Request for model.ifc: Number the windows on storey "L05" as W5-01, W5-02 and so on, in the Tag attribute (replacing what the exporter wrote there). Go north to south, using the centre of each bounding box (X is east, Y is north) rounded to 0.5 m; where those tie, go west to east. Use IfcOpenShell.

First a look at what the model holds.

```python
import ifcopenshell
import ifcopenshell.util.element
import ifcopenshell.util.placement

model = ifcopenshell.open("model.ifc")
print(model.schema)
storey = next(s for s in model.by_type("IfcBuildingStorey") if s.Name == "L05")
windows = [e for e in ifcopenshell.util.element.get_decomposition(storey) if e.is_a("IfcWindow")]
for e in sorted(windows, key=lambda e: e.id()):
    origin = ifcopenshell.util.placement.get_local_placement(e.ObjectPlacement)[:3, 3]
    print(e.id(), e.Tag, e.Name, origin.round(2) + 0.0, sep=" | ")
```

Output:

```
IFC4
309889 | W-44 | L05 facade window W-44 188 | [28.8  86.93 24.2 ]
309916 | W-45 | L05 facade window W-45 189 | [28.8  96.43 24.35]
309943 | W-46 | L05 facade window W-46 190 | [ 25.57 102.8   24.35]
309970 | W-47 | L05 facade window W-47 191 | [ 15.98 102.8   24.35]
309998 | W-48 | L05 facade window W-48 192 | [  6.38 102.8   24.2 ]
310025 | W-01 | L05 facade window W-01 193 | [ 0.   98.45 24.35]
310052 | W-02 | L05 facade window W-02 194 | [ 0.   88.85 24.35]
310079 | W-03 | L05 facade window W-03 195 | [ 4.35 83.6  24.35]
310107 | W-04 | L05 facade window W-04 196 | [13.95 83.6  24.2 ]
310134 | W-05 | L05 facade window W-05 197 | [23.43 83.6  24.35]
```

```python
import ifcopenshell
import ifcopenshell.geom
import ifcopenshell.util.element
import ifcopenshell.util.shape

model = ifcopenshell.open("model.ifc")
settings = ifcopenshell.geom.settings()
settings.set("use-world-coords", True)


def centre(element):
    shape = ifcopenshell.geom.create_shape(settings, element)
    return ifcopenshell.util.shape.get_bbox_centroid(shape.geometry)


storey = next(s for s in model.by_type("IfcBuildingStorey") if s.Name == "L05")
windows = [e for e in ifcopenshell.util.element.get_decomposition(storey) if e.is_a("IfcWindow")]

# Insertion points can sit at a corner or the storey origin, so sort by the geometry (in metres).
centres = {e: centre(e) for e in windows}
windows.sort(key=lambda e: (-round(centres[e][1] / 0.5), centres[e][0]))

for i, e in enumerate(windows, start=1):
    number = f"W5-{i:02d}"
    e.Tag = number
    print(e.id(), number)

model.write("model-out.ifc")
```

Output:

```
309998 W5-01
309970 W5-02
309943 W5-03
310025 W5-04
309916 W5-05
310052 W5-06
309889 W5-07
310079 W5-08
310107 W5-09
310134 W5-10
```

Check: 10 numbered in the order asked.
